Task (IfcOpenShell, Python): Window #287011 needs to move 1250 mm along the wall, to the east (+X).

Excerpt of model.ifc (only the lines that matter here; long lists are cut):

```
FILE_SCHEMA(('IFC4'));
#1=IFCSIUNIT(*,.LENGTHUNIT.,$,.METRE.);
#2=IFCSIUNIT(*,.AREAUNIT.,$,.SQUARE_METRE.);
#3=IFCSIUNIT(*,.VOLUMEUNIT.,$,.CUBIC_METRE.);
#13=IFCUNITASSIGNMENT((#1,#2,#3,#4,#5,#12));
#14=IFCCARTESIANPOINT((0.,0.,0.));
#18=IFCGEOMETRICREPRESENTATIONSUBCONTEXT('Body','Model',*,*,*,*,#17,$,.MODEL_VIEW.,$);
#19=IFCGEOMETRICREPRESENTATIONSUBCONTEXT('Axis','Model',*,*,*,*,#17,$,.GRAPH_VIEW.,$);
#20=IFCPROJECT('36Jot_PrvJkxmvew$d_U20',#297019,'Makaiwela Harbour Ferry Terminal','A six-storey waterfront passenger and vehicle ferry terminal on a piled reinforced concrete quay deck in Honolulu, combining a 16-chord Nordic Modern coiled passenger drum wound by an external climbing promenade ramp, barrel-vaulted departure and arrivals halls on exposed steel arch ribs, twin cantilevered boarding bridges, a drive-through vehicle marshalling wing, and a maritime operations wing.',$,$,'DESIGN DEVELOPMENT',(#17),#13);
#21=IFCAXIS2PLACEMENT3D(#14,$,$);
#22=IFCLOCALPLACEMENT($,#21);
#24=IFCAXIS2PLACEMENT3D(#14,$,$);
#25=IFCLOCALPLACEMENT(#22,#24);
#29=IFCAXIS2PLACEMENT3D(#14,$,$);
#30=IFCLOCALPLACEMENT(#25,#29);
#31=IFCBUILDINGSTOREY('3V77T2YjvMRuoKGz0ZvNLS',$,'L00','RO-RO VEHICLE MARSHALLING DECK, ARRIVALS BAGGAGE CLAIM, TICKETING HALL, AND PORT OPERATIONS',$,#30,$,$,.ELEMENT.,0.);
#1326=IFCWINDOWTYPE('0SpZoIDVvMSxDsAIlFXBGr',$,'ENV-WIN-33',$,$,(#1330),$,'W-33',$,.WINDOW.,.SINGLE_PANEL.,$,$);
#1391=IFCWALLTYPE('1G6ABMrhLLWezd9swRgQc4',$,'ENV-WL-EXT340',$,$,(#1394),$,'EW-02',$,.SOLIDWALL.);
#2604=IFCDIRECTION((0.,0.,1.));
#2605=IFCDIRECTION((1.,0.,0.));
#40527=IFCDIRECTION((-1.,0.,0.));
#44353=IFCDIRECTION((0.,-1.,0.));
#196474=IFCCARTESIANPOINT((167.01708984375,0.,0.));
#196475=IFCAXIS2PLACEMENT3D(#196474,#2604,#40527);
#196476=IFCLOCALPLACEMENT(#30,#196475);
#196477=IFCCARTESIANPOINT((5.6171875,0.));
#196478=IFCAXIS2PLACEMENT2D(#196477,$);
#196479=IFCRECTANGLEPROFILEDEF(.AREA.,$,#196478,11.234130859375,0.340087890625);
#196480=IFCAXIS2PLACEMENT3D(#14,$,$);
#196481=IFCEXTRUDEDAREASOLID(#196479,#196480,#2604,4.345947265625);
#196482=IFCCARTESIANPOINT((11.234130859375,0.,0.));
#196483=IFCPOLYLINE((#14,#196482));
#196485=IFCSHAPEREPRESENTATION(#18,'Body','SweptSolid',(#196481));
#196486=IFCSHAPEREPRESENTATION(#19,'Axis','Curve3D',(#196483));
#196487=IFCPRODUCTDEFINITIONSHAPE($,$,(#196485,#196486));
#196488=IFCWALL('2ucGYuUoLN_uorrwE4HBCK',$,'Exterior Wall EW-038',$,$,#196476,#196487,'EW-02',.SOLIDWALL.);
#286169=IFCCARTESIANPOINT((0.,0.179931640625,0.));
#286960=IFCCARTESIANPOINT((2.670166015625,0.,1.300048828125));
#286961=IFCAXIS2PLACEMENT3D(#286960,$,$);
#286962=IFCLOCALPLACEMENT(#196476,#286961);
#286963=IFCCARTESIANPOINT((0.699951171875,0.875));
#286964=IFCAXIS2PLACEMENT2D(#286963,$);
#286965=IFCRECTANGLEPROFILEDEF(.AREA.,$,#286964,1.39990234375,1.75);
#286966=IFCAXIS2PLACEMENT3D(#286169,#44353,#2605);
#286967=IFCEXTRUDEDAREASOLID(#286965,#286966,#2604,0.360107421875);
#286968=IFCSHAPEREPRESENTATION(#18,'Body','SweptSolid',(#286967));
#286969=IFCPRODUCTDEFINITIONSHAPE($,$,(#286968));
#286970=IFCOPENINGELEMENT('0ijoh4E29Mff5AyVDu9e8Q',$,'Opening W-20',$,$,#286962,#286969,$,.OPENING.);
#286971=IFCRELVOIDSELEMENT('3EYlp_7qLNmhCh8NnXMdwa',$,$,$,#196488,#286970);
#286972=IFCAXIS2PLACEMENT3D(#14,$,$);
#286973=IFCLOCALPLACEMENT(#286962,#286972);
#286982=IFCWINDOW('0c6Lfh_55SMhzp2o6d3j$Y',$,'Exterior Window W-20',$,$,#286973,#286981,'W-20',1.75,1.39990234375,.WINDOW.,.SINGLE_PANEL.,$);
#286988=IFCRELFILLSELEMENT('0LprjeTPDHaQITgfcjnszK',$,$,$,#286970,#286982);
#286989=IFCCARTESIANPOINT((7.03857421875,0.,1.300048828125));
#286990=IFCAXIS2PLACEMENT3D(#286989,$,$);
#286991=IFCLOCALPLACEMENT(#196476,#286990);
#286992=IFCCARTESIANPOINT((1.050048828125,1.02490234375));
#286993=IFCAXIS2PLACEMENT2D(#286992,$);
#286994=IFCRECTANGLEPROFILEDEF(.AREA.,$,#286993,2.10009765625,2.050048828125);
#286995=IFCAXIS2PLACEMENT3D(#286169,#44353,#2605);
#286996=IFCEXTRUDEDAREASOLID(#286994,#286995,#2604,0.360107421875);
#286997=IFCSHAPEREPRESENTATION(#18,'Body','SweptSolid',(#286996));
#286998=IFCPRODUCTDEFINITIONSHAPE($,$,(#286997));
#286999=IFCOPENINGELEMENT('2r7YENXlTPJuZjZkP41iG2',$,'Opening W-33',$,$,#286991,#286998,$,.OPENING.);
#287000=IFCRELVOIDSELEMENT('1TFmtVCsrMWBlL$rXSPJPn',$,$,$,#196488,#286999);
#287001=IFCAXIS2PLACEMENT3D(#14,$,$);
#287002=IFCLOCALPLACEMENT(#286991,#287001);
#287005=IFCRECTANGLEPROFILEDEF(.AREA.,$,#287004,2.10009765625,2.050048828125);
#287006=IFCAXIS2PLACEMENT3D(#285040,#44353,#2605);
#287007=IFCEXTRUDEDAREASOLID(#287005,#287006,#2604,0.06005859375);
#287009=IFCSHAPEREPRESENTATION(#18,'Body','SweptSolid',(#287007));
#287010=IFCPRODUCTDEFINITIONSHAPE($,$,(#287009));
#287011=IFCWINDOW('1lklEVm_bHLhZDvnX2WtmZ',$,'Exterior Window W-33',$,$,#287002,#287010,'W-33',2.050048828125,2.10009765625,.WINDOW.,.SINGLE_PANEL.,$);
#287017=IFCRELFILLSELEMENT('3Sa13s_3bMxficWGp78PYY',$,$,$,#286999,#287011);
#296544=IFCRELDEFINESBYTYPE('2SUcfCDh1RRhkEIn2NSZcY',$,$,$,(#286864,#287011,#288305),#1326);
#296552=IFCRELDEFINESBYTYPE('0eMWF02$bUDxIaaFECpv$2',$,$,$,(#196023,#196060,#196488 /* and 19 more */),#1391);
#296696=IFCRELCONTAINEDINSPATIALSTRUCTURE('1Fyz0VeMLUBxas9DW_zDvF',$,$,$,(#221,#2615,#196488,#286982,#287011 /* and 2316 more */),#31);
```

```python
import ifcopenshell
import ifcopenshell.api.geometry
import ifcopenshell.util.placement
import ifcopenshell.util.unit

model = ifcopenshell.open("model.ifc")
unit_scale = ifcopenshell.util.unit.calculate_unit_scale(model)

window = model.by_guid("1lklEVm_bHLhZDvnX2WtmZ")
opening = window.FillsVoids[0].RelatingOpeningElement
wall = opening.VoidsElements[0].RelatingBuildingElement

wall_matrix = ifcopenshell.util.placement.get_local_placement(wall.ObjectPlacement)
shift = wall_matrix[:3, 0] * -1.25 / unit_scale
before = ifcopenshell.util.placement.get_local_placement(window.ObjectPlacement)[:3, 3].copy()

# The window is placed relative to its opening, so it follows when the opening moves.
matrix = ifcopenshell.util.placement.get_local_placement(opening.ObjectPlacement)
matrix[:3, 3] += shift
ifcopenshell.api.geometry.edit_object_placement(
    model, product=opening, matrix=matrix, is_si=False, should_transform_children=True
)

after = ifcopenshell.util.placement.get_local_placement(window.ObjectPlacement)[:3, 3]
print("window moved by", (after - before).round(3) + 0.0)

model.write("model_updated.ifc")
```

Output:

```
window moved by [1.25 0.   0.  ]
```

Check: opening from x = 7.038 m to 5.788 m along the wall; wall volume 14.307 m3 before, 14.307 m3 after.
